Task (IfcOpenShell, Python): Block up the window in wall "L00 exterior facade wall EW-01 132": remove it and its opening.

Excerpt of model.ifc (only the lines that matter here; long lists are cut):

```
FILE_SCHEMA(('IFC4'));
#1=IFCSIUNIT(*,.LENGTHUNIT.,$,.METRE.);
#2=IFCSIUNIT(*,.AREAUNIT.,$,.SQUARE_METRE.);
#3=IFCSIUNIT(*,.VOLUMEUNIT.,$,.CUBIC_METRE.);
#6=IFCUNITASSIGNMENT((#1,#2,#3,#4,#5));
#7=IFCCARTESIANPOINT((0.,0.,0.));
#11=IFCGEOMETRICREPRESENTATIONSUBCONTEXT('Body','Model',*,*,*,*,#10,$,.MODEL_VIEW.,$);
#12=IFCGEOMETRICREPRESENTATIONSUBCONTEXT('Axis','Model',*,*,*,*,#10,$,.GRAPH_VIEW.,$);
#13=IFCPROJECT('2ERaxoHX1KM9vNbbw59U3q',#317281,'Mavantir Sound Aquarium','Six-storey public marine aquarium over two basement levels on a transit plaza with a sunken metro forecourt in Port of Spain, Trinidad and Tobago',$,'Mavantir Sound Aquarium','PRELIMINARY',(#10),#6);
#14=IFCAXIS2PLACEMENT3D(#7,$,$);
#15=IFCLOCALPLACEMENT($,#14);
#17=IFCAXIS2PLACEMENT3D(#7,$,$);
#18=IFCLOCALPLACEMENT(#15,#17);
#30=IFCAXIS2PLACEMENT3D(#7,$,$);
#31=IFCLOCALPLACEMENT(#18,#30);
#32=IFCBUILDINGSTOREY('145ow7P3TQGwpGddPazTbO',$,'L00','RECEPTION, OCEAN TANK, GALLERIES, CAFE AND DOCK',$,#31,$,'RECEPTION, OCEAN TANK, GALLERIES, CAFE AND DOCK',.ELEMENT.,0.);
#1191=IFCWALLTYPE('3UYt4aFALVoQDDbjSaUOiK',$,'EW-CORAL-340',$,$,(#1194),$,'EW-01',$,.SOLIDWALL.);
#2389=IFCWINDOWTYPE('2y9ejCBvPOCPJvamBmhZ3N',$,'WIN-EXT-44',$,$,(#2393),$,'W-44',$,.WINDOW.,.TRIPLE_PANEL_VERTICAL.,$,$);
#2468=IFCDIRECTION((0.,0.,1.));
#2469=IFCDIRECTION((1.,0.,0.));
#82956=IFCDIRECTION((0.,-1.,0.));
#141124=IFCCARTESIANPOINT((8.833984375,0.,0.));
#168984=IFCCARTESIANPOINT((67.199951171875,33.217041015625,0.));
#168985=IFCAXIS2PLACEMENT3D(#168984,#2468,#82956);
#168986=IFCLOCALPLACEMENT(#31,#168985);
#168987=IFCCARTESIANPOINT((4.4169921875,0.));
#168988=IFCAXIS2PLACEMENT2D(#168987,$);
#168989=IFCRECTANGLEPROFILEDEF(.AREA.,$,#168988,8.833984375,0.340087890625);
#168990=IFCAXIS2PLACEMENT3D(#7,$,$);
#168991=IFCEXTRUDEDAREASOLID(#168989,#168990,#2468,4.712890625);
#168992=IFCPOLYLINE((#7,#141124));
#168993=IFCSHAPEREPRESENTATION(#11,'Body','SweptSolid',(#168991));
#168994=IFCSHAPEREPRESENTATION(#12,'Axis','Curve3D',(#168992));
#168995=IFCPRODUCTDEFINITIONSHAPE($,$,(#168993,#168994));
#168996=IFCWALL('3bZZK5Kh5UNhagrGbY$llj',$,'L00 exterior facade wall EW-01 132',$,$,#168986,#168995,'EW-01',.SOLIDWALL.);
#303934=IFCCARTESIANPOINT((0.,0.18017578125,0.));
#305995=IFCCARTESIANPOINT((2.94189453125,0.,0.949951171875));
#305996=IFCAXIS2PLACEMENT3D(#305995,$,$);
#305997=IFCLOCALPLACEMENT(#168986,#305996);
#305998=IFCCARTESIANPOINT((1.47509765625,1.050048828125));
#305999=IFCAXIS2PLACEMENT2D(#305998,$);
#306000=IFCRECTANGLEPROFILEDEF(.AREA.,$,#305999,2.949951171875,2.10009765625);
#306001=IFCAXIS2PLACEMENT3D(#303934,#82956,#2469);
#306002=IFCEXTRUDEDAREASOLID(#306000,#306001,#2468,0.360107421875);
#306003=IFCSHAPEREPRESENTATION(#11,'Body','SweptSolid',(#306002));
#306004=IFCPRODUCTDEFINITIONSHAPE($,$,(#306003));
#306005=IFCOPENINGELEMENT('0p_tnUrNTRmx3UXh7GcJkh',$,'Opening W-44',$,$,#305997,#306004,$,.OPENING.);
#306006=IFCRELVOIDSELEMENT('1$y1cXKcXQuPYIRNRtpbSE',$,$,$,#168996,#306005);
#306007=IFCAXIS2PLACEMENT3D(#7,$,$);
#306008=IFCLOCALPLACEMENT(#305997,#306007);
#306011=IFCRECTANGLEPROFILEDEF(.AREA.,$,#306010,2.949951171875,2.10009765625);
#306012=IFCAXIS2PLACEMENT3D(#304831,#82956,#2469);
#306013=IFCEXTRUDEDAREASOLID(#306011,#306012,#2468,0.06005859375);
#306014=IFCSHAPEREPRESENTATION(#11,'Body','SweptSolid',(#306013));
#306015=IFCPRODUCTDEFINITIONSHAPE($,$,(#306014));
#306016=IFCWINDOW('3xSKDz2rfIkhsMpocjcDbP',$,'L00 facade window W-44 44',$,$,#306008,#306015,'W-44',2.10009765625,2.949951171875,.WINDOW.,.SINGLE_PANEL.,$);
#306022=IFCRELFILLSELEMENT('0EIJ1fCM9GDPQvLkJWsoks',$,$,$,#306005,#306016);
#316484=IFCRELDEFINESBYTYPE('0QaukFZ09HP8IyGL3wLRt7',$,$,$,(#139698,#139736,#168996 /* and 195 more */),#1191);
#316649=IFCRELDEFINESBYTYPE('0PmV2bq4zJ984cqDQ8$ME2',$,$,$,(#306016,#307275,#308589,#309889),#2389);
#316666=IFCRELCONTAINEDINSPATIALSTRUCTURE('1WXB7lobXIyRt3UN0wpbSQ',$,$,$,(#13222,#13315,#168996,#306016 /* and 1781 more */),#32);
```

```python
import ifcopenshell
import ifcopenshell.api.feature
import ifcopenshell.api.root
import ifcopenshell.geom
import ifcopenshell.util.shape

model = ifcopenshell.open("model.ifc")
settings = ifcopenshell.geom.settings()


def volume(element):
    """Net volume in cubic metres, openings subtracted."""
    shape = ifcopenshell.geom.create_shape(settings, element)
    return ifcopenshell.util.shape.get_volume(shape.geometry)


window = model.by_guid("3xSKDz2rfIkhsMpocjcDbP")
opening = window.FillsVoids[0].RelatingOpeningElement
wall = opening.VoidsElements[0].RelatingBuildingElement
before = volume(wall)

ifcopenshell.api.root.remove_product(model, product=window)
ifcopenshell.api.feature.remove_feature(model, feature=opening)

after = volume(wall)

print(f"wall volume {before:.3f} -> {after:.3f} m3")

model.write("model-out.ifc")
```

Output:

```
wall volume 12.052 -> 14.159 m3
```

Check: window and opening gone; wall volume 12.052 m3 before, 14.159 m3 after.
